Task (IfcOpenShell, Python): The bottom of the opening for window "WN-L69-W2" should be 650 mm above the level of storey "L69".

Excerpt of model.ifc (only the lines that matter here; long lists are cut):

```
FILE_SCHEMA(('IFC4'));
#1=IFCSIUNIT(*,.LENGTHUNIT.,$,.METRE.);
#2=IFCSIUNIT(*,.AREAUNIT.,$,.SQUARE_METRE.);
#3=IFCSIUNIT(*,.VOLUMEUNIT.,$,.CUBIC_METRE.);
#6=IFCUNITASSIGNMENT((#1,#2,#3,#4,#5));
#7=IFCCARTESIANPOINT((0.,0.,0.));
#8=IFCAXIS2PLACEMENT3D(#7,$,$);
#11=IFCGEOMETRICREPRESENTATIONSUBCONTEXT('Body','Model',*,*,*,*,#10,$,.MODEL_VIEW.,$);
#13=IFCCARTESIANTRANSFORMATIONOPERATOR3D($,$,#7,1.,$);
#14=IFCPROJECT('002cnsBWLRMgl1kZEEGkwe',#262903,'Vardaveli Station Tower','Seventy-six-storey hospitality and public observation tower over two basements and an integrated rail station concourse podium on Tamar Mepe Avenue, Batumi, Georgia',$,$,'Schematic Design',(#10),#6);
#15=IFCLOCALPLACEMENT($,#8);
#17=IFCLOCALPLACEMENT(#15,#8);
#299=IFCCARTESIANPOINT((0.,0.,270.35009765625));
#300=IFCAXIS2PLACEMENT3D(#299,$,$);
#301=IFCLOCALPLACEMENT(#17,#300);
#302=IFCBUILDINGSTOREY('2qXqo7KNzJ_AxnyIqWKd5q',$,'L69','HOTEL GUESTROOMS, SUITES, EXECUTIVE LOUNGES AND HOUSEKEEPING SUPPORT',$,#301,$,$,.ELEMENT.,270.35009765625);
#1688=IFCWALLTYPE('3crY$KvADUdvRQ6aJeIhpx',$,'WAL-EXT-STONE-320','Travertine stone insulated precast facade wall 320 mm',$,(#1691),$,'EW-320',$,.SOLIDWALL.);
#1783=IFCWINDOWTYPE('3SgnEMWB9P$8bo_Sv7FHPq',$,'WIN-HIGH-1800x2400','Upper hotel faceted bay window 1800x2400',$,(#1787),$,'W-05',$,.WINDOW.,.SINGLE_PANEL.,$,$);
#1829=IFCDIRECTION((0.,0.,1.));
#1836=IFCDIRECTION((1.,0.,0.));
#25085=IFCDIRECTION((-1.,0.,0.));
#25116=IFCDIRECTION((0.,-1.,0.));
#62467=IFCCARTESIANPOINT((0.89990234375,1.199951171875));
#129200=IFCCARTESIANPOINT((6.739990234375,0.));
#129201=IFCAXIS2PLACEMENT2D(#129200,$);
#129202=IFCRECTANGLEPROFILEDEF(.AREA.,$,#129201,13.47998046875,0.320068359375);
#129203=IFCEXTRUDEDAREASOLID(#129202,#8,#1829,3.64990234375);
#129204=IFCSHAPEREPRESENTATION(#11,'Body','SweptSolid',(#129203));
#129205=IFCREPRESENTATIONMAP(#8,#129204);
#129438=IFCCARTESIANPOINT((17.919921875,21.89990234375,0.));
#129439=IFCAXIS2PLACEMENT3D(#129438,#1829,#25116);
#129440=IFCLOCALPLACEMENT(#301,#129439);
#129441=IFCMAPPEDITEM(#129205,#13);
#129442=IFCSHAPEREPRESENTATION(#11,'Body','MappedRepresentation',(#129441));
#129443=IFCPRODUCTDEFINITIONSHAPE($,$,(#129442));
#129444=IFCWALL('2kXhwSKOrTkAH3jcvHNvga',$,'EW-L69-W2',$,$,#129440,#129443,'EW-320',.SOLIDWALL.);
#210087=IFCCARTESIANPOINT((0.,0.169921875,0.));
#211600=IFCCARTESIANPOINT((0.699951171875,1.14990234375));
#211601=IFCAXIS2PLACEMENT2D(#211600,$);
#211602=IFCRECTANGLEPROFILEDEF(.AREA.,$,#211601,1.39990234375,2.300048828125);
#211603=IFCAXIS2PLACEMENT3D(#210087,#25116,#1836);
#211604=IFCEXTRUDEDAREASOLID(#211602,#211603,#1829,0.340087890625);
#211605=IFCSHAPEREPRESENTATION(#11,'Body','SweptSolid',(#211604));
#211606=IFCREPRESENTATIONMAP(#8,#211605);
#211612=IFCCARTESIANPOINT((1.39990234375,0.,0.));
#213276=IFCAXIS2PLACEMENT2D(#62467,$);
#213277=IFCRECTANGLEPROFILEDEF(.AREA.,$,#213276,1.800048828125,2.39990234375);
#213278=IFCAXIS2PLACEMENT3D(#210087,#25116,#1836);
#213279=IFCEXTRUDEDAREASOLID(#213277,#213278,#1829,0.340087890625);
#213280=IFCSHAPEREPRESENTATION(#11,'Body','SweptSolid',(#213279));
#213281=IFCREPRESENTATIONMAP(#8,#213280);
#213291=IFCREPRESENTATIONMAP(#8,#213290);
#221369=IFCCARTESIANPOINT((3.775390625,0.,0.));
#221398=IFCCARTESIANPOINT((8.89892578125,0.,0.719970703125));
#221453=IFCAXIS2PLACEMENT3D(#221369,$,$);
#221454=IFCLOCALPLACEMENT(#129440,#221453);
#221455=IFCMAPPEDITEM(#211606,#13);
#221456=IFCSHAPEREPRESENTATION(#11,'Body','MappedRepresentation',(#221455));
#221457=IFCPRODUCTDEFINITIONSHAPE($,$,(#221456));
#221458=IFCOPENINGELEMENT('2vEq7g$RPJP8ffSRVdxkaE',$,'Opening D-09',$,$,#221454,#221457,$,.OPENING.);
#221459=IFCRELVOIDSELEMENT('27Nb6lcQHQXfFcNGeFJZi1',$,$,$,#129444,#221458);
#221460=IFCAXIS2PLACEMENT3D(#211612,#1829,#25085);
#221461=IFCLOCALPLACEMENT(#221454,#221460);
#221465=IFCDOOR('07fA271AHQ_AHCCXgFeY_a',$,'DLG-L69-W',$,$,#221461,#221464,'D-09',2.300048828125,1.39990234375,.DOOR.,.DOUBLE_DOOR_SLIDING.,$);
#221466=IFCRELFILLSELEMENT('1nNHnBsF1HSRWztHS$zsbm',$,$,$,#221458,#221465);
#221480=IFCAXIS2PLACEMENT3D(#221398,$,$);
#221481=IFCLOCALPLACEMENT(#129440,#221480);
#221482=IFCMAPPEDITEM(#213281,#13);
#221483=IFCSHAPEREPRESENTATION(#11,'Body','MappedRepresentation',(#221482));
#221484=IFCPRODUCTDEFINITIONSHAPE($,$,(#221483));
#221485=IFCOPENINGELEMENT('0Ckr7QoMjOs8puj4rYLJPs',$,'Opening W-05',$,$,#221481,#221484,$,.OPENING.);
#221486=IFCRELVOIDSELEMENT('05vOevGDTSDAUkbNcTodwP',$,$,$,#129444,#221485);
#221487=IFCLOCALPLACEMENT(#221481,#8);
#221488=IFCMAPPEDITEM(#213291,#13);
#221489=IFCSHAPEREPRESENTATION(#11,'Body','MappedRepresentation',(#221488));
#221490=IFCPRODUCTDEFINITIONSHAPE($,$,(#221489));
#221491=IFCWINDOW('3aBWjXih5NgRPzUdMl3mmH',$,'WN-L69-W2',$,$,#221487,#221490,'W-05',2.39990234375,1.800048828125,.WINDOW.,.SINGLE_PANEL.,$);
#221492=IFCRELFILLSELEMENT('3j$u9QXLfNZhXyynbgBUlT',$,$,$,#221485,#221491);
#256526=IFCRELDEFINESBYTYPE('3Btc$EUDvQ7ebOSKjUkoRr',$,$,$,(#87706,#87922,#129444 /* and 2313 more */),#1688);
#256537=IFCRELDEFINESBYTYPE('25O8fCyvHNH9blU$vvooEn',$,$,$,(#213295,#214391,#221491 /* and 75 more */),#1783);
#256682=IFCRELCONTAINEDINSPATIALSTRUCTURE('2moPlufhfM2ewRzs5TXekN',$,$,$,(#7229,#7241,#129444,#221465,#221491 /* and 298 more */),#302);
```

```python
import numpy as np
import ifcopenshell
import ifcopenshell.api.geometry
import ifcopenshell.geom
import ifcopenshell.util.element
import ifcopenshell.util.placement
import ifcopenshell.util.shape
import ifcopenshell.util.unit

model = ifcopenshell.open("model.ifc")
unit_scale = ifcopenshell.util.unit.calculate_unit_scale(model)

window = model.by_id(221491)
opening = window.FillsVoids[0].RelatingOpeningElement
storey = ifcopenshell.util.element.get_container(window, ifc_class="IfcBuildingStorey")
level = ifcopenshell.util.placement.get_local_placement(storey.ObjectPlacement)[2, 3]

# The opening's origin need not be at the sill, so measure its lowest point.
shape = ifcopenshell.geom.create_shape(ifcopenshell.geom.settings(), opening)
bottom = ifcopenshell.util.shape.get_shape_bottom_elevation(shape, shape.geometry) / unit_scale
dz = level + 0.65 - bottom

shift = np.array([0.0, 0.0, dz])
# The window is placed relative to its opening, so it follows when the opening moves.
matrix = ifcopenshell.util.placement.get_local_placement(opening.ObjectPlacement)
matrix[:3, 3] += shift
ifcopenshell.api.geometry.edit_object_placement(
    model, product=opening, matrix=matrix, is_si=False, should_transform_children=True
)

print(f"moved by {dz * unit_scale:+.3f} m")

model.write("model_rev.ifc")
```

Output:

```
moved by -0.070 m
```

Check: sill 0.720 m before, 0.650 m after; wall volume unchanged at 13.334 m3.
